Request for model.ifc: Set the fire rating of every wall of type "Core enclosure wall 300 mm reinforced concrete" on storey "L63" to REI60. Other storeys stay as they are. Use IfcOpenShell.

First a look at what the model holds.

```python
import ifcopenshell
import ifcopenshell.util.element

model = ifcopenshell.open("model.ifc")
print(model.schema)
storey = next(s for s in model.by_type("IfcBuildingStorey") if s.Name == "L63")
walls = [e for e in ifcopenshell.util.element.get_decomposition(storey) if e.is_a("IfcWall")]
seen = {}
for e in walls:
    element_type = ifcopenshell.util.element.get_type(e)
    key = (element_type.Name if element_type != e and element_type else None, ifcopenshell.util.element.get_pset(e, "Pset_WallCommon", "FireRating"))
    seen[key] = seen.get(key, 0) + 1
for (name, value), count in sorted(seen.items(), key=str):
    print(count, "x", name, "|", value)
```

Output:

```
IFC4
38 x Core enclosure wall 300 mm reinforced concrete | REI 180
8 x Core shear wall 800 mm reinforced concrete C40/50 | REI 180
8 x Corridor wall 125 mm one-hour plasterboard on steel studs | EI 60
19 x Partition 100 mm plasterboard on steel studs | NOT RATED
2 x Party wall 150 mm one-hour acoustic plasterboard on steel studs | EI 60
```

```python
import ifcopenshell
import ifcopenshell.api.pset
import ifcopenshell.util.element

model = ifcopenshell.open("model.ifc")

storey = next(s for s in model.by_type("IfcBuildingStorey") if s.Name == "L63")
walls = [e for e in ifcopenshell.util.element.get_decomposition(storey) if e.is_a("IfcWall")]

count = 0
for e in walls:
    element_type = ifcopenshell.util.element.get_type(e)
    if element_type in (None, e) or element_type.Name != "Core enclosure wall 300 mm reinforced concrete":
        continue
    found = ifcopenshell.util.element.get_pset(e, "Pset_WallCommon", should_inherit=False)
    if found:
        pset = model.by_id(found["id"])
        if len(ifcopenshell.util.element.get_elements_by_pset(pset)) > 1:
            pset = ifcopenshell.api.pset.unshare_pset(model, products=[e], pset=pset)[0]
    else:
        pset = ifcopenshell.api.pset.add_pset(model, product=e, name="Pset_WallCommon")
    ifcopenshell.api.pset.edit_pset(model, pset=pset, properties={"FireRating": "REI60"})
    count += 1

print(count, "walls updated")

model.write("model_rev.ifc")
```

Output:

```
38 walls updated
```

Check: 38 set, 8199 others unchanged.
